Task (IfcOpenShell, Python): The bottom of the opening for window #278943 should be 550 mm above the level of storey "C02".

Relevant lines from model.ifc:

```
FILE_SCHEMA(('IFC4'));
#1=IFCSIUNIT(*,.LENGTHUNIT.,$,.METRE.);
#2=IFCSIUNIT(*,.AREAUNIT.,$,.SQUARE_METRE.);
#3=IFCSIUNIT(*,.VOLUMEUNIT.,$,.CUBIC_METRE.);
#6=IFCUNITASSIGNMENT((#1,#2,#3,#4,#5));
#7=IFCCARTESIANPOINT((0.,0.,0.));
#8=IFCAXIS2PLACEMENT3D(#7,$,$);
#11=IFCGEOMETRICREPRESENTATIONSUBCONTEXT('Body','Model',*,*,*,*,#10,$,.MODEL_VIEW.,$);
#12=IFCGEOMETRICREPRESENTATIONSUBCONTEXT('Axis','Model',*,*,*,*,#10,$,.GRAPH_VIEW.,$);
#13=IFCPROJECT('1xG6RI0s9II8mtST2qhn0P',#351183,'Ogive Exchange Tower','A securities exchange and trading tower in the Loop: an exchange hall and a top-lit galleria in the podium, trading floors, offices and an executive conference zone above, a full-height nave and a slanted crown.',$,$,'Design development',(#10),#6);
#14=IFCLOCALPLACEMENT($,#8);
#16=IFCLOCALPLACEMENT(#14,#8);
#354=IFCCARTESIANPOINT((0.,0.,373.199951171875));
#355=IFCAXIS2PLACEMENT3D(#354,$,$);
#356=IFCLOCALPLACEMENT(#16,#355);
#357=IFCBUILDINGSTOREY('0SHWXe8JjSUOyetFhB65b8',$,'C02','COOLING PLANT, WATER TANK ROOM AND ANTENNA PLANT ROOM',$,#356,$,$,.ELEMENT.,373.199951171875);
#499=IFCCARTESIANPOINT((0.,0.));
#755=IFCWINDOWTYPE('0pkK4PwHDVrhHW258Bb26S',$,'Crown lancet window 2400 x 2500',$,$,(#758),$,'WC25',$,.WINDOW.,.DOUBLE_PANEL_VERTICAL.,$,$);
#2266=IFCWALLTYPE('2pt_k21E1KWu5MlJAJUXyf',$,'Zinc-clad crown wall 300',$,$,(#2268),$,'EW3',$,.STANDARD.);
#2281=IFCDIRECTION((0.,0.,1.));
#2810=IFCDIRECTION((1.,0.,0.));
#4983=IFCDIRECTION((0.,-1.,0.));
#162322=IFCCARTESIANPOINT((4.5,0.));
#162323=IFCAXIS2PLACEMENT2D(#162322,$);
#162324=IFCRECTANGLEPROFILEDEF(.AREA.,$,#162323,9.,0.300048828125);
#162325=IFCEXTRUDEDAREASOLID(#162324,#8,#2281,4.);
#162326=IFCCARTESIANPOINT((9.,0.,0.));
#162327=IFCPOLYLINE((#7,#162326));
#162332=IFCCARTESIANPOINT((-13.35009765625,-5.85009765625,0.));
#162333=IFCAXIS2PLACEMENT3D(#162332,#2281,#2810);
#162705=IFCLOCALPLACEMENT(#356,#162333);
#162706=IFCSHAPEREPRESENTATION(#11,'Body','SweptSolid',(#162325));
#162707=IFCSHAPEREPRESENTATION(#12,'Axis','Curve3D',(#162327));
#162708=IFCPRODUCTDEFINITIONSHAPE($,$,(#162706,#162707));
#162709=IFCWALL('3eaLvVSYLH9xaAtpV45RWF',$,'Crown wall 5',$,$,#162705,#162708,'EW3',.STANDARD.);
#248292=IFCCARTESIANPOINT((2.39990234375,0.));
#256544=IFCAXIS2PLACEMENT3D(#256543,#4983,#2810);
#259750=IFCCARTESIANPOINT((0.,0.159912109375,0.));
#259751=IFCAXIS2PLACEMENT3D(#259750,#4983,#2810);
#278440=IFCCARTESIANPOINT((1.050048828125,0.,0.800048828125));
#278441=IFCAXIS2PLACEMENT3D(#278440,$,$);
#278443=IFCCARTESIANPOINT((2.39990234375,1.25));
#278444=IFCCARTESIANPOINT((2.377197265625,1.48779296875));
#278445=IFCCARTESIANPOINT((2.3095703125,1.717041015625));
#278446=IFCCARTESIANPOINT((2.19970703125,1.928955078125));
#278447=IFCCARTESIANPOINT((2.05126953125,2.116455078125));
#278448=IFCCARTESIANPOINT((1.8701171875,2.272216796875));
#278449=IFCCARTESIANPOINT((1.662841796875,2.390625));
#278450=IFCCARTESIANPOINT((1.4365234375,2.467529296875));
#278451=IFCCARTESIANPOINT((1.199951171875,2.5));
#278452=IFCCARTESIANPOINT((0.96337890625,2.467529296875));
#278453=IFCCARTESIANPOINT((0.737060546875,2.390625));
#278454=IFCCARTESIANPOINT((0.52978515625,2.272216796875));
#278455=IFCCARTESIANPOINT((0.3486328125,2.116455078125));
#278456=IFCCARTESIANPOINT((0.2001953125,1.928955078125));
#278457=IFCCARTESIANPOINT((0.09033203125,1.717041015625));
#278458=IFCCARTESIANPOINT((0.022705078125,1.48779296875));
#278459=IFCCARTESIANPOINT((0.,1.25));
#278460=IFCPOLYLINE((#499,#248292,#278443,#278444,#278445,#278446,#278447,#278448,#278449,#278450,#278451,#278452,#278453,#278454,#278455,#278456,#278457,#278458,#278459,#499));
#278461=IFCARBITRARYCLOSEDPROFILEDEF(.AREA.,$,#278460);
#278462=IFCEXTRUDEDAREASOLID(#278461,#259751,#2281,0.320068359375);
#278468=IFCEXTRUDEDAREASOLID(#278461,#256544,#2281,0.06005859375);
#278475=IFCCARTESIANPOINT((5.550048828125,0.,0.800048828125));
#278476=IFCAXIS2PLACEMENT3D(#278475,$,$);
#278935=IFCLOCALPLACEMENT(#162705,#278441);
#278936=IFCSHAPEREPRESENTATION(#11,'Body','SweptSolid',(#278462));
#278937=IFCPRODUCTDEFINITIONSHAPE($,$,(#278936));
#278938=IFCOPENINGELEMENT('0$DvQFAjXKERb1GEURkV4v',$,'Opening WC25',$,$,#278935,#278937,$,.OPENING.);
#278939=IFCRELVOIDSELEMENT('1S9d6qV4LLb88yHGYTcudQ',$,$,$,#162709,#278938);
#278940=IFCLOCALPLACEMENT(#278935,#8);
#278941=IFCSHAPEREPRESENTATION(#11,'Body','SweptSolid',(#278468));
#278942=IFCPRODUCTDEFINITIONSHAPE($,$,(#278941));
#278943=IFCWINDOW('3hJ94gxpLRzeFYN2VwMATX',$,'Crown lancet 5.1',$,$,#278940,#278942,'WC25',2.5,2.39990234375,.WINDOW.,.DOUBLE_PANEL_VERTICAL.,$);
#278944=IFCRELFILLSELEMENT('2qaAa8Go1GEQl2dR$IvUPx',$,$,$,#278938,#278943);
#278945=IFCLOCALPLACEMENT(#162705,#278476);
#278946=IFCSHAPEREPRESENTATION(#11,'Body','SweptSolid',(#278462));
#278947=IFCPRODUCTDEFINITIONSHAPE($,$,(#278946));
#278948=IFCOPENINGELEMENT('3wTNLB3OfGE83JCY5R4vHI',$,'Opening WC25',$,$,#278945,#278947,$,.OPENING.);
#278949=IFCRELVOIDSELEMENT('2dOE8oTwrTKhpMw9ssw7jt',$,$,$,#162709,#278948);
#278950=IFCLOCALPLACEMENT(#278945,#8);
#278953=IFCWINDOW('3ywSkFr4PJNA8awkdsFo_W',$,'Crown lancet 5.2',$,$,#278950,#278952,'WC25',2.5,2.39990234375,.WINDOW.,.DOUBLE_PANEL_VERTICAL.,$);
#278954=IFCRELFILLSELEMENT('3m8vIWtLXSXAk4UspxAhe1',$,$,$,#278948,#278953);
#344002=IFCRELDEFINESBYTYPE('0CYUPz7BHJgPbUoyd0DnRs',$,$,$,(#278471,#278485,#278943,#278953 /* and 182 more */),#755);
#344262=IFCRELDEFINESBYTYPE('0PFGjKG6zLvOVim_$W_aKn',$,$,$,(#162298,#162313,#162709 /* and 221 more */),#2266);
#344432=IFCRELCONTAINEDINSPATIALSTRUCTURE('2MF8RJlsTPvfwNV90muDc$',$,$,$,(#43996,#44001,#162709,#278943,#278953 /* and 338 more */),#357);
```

```python
import numpy as np
import ifcopenshell
import ifcopenshell.api.geometry
import ifcopenshell.geom
import ifcopenshell.util.element
import ifcopenshell.util.placement
import ifcopenshell.util.shape
import ifcopenshell.util.unit

model = ifcopenshell.open("model.ifc")
unit_scale = ifcopenshell.util.unit.calculate_unit_scale(model)

window = model.by_guid("3hJ94gxpLRzeFYN2VwMATX")
opening = window.FillsVoids[0].RelatingOpeningElement
storey = ifcopenshell.util.element.get_container(window, ifc_class="IfcBuildingStorey")
level = ifcopenshell.util.placement.get_local_placement(storey.ObjectPlacement)[2, 3]

# The opening's origin need not be at the sill, so measure its lowest point.
shape = ifcopenshell.geom.create_shape(ifcopenshell.geom.settings(), opening)
bottom = ifcopenshell.util.shape.get_shape_bottom_elevation(shape, shape.geometry) / unit_scale
dz = level + 0.55 / unit_scale - bottom

shift = np.array([0.0, 0.0, dz])
# The window is placed relative to its opening, so it follows when the opening moves.
matrix = ifcopenshell.util.placement.get_local_placement(opening.ObjectPlacement)
matrix[:3, 3] += shift
ifcopenshell.api.geometry.edit_object_placement(
    model, product=opening, matrix=matrix, is_si=False, should_transform_children=True
)

print(f"moved by {dz * unit_scale:+.3f} m")

model.write("model_updated.ifc")
```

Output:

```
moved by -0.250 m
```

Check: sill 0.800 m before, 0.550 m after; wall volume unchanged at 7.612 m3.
